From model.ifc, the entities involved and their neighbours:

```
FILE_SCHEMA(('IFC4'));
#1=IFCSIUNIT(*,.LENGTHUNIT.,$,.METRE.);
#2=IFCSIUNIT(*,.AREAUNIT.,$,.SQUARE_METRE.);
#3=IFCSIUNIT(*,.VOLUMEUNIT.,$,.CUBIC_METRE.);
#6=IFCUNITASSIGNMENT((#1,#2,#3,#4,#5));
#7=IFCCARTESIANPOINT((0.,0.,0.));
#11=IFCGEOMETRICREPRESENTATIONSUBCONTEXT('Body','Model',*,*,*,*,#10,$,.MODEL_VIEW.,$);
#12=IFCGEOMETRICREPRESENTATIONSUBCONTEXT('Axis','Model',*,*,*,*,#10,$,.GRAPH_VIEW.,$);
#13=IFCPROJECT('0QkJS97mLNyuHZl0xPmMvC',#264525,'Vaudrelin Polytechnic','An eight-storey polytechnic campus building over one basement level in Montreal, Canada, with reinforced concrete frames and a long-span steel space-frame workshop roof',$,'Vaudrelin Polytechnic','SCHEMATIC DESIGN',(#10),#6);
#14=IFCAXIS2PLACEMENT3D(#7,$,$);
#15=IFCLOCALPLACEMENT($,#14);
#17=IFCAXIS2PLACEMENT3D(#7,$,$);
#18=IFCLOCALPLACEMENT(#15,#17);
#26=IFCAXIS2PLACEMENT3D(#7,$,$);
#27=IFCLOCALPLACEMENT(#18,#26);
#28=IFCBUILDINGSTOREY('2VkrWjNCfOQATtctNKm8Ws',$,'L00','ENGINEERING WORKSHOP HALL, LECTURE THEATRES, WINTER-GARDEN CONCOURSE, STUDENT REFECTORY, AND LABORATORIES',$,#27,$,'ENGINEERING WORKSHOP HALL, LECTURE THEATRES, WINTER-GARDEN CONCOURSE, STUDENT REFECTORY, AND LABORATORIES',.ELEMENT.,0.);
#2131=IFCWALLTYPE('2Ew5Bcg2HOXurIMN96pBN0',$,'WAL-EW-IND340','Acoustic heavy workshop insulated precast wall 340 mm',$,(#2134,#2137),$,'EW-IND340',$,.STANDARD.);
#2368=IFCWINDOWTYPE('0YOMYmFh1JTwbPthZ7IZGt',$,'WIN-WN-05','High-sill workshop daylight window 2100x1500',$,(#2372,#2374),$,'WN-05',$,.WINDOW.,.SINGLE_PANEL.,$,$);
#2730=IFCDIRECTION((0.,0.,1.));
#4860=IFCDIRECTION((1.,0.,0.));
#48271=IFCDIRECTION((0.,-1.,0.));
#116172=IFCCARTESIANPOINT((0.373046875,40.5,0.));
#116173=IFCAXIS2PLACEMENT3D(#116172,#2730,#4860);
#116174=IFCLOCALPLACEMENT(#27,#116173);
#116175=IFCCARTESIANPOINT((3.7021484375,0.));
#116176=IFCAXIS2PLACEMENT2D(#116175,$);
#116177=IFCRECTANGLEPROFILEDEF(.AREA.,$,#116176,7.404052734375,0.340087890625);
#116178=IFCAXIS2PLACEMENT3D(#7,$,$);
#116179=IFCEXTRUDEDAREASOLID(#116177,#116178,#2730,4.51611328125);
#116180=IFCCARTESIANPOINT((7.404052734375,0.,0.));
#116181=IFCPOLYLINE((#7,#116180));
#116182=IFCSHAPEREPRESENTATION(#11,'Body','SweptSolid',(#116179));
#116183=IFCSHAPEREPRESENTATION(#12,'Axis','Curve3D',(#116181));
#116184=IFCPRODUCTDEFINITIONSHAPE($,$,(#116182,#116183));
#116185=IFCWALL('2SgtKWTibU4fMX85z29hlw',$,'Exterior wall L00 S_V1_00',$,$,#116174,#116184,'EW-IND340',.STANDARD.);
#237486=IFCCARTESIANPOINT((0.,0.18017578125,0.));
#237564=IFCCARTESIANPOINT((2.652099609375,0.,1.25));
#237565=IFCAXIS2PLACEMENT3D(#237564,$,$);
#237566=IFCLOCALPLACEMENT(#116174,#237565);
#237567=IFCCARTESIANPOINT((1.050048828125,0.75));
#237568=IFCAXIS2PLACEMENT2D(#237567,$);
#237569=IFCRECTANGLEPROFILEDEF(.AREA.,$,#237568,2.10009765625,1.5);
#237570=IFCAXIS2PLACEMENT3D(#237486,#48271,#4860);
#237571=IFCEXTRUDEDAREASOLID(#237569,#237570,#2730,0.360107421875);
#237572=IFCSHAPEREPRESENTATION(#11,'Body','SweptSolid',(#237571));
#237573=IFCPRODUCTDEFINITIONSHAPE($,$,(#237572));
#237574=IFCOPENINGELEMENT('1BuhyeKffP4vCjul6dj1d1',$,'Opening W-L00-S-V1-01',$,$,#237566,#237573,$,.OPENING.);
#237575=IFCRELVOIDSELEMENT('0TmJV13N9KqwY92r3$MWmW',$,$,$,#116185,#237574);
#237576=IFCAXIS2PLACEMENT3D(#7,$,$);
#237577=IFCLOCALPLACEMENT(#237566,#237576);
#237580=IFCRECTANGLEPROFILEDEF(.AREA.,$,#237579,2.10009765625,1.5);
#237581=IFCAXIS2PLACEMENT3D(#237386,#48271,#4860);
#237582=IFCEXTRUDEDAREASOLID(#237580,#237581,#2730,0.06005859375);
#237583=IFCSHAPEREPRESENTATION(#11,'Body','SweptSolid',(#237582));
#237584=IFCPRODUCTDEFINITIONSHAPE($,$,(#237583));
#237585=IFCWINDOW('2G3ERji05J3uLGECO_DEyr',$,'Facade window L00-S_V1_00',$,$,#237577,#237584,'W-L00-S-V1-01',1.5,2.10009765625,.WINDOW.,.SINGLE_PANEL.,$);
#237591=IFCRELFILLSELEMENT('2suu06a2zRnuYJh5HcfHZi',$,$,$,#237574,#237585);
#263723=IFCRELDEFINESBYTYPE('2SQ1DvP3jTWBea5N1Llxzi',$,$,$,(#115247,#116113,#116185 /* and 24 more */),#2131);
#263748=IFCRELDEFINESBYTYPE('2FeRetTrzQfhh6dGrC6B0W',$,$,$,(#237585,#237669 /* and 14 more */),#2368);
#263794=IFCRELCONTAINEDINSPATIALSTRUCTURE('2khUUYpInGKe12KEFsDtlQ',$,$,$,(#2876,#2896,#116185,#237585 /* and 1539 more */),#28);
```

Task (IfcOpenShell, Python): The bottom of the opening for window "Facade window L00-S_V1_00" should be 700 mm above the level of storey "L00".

```python
import numpy as np
import ifcopenshell
import ifcopenshell.api.geometry
import ifcopenshell.geom
import ifcopenshell.util.element
import ifcopenshell.util.placement
import ifcopenshell.util.shape
import ifcopenshell.util.unit

model = ifcopenshell.open("model.ifc")
unit_scale = ifcopenshell.util.unit.calculate_unit_scale(model)

window = model.by_guid("2G3ERji05J3uLGECO_DEyr")
opening = window.FillsVoids[0].RelatingOpeningElement
storey = ifcopenshell.util.element.get_container(window, ifc_class="IfcBuildingStorey")
level = ifcopenshell.util.placement.get_local_placement(storey.ObjectPlacement)[2, 3]

# The opening's origin need not be at the sill, so measure its lowest point.
shape = ifcopenshell.geom.create_shape(ifcopenshell.geom.settings(), opening)
bottom = ifcopenshell.util.shape.get_shape_bottom_elevation(shape, shape.geometry) / unit_scale
dz = level + 0.7 - bottom

shift = np.array([0.0, 0.0, dz])
# The window is placed relative to its opening, so it follows when the opening moves.
matrix = ifcopenshell.util.placement.get_local_placement(opening.ObjectPlacement)
matrix[:3, 3] += shift
ifcopenshell.api.geometry.edit_object_placement(
    model, product=opening, matrix=matrix, is_si=False, should_transform_children=True
)

print(f"moved by {dz * unit_scale:+.3f} m")

model.write("model_edited.ifc")
```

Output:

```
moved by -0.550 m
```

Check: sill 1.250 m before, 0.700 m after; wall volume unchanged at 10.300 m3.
